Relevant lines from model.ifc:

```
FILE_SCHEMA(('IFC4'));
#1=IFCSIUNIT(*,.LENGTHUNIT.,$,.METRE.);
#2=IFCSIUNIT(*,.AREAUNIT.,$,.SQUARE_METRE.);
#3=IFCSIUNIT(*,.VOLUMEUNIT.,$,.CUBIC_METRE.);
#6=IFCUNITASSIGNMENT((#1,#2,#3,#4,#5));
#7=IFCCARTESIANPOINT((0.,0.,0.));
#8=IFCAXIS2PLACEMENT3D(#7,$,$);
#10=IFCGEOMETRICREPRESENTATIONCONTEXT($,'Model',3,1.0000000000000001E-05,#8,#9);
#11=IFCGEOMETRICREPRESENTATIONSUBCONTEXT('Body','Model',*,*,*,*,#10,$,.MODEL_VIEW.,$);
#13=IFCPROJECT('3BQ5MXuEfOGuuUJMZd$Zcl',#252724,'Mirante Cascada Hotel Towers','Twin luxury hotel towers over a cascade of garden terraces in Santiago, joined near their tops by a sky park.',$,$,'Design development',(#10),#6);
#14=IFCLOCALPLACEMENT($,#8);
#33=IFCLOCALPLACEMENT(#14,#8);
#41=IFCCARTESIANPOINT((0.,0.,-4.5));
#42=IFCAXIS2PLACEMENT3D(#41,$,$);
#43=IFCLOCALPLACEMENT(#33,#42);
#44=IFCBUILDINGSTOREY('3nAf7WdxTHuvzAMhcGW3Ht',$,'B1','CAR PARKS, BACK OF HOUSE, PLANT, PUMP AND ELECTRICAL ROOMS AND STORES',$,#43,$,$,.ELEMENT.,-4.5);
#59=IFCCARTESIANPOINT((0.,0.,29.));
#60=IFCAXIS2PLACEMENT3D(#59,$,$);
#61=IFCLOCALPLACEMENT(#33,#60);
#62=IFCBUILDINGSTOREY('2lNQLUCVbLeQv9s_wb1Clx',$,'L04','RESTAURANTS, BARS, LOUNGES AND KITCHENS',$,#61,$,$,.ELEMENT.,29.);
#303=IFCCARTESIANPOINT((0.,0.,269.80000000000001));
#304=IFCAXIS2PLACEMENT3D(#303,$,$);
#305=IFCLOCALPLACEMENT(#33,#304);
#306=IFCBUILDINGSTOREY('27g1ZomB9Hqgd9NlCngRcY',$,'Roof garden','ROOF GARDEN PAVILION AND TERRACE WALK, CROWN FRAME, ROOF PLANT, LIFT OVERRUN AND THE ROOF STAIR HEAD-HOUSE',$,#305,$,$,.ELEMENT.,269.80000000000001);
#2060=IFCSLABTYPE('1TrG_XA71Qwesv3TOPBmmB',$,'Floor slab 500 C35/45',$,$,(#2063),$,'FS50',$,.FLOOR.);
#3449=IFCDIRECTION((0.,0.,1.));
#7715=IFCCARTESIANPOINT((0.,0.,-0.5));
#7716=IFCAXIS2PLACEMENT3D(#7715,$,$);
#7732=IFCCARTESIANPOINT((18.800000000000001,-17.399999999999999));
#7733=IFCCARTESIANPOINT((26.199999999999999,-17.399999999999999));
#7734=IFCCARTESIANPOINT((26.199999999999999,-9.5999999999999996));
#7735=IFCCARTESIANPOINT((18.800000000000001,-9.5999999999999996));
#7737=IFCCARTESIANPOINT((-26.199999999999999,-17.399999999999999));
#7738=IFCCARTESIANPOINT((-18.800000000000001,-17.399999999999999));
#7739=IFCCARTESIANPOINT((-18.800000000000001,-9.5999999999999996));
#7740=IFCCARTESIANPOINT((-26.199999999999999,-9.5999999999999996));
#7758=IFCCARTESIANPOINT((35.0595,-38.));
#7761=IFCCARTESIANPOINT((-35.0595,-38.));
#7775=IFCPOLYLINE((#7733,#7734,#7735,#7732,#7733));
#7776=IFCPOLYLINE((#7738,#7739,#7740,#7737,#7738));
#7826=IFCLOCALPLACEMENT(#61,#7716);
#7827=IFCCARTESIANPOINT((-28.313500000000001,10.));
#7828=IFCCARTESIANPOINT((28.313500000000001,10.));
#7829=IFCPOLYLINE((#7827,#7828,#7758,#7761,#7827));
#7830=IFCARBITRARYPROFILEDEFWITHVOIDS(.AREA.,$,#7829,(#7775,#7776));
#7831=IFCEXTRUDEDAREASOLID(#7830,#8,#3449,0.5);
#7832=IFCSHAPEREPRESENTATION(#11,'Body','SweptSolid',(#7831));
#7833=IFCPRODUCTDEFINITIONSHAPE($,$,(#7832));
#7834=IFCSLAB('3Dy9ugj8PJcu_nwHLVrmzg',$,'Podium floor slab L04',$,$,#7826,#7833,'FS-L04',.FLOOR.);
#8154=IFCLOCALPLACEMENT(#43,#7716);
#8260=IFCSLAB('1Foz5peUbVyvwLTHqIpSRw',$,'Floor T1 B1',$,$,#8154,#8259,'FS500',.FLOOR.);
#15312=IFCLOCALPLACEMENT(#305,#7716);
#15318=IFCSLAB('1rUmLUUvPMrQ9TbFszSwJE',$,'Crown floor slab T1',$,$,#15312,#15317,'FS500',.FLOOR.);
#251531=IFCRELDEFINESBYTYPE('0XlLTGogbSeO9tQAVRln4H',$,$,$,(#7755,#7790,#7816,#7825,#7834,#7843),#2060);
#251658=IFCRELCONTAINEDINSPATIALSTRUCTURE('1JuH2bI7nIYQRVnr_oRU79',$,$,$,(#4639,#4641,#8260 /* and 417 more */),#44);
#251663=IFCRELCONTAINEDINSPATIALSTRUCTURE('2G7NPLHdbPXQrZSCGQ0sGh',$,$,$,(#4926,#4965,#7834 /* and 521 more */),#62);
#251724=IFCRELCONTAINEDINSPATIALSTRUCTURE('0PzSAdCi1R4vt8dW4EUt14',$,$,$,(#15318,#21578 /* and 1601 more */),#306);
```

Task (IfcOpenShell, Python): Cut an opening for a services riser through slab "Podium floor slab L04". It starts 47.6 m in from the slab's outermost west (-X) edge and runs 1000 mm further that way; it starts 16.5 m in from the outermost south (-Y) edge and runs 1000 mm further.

```python
import numpy as np
import ifcopenshell
import ifcopenshell.api.feature
import ifcopenshell.api.geometry
import ifcopenshell.api.root
import ifcopenshell.geom
import ifcopenshell.util.placement
import ifcopenshell.util.representation
import ifcopenshell.util.shape
import ifcopenshell.util.unit

model = ifcopenshell.open("model.ifc")
unit_scale = ifcopenshell.util.unit.calculate_unit_scale(model)
settings = ifcopenshell.geom.settings()


def volume(element):
    """Net volume in cubic metres, openings subtracted."""
    shape = ifcopenshell.geom.create_shape(settings, element)
    return ifcopenshell.util.shape.get_volume(shape.geometry)


slab = model.by_guid("3Dy9ugj8PJcu_nwHLVrmzg")
before = volume(slab)

# Extent in the slab's own axes, in metres. The edges named are its -X and -Y sides.
slab_shape = ifcopenshell.geom.create_shape(settings, slab)
vertices = ifcopenshell.util.shape.get_vertices(slab_shape.geometry)
x_min, y_min, bottom = vertices.min(axis=0)
top = vertices[:, 2].max()

opening = ifcopenshell.api.root.create_entity(model, ifc_class="IfcOpeningElement", name="Services riser opening", predefined_type="OPENING")
context = ifcopenshell.util.representation.get_context(model, "Model", "Body", "MODEL_VIEW")
width, depth = 1, 1
outline = [(0.0, 0.0), (width, 0.0), (width, depth), (0.0, depth), (0.0, 0.0)]
# Overshoot both faces by 50 mm so the cut is clean.
shape = ifcopenshell.api.geometry.add_slab_representation(
    model, context=context, depth=top - bottom + 0.1, polyline=outline
)
ifcopenshell.api.geometry.assign_representation(model, product=opening, representation=shape)

matrix = ifcopenshell.util.placement.get_local_placement(slab.ObjectPlacement)
matrix[:, 3] = matrix @ np.append(np.array([x_min + 47.6, y_min + 16.5, bottom - 0.05]) / unit_scale, 1.0)
ifcopenshell.api.geometry.edit_object_placement(model, product=opening, matrix=matrix, is_si=False)
ifcopenshell.api.feature.add_feature(model, feature=opening, element=slab)

after = volume(slab)

print(f"slab volume {before:.3f} -> {after:.3f} m3")

model.write("model-out.ifc")
```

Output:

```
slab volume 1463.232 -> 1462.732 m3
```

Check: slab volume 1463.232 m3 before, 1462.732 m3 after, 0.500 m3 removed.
